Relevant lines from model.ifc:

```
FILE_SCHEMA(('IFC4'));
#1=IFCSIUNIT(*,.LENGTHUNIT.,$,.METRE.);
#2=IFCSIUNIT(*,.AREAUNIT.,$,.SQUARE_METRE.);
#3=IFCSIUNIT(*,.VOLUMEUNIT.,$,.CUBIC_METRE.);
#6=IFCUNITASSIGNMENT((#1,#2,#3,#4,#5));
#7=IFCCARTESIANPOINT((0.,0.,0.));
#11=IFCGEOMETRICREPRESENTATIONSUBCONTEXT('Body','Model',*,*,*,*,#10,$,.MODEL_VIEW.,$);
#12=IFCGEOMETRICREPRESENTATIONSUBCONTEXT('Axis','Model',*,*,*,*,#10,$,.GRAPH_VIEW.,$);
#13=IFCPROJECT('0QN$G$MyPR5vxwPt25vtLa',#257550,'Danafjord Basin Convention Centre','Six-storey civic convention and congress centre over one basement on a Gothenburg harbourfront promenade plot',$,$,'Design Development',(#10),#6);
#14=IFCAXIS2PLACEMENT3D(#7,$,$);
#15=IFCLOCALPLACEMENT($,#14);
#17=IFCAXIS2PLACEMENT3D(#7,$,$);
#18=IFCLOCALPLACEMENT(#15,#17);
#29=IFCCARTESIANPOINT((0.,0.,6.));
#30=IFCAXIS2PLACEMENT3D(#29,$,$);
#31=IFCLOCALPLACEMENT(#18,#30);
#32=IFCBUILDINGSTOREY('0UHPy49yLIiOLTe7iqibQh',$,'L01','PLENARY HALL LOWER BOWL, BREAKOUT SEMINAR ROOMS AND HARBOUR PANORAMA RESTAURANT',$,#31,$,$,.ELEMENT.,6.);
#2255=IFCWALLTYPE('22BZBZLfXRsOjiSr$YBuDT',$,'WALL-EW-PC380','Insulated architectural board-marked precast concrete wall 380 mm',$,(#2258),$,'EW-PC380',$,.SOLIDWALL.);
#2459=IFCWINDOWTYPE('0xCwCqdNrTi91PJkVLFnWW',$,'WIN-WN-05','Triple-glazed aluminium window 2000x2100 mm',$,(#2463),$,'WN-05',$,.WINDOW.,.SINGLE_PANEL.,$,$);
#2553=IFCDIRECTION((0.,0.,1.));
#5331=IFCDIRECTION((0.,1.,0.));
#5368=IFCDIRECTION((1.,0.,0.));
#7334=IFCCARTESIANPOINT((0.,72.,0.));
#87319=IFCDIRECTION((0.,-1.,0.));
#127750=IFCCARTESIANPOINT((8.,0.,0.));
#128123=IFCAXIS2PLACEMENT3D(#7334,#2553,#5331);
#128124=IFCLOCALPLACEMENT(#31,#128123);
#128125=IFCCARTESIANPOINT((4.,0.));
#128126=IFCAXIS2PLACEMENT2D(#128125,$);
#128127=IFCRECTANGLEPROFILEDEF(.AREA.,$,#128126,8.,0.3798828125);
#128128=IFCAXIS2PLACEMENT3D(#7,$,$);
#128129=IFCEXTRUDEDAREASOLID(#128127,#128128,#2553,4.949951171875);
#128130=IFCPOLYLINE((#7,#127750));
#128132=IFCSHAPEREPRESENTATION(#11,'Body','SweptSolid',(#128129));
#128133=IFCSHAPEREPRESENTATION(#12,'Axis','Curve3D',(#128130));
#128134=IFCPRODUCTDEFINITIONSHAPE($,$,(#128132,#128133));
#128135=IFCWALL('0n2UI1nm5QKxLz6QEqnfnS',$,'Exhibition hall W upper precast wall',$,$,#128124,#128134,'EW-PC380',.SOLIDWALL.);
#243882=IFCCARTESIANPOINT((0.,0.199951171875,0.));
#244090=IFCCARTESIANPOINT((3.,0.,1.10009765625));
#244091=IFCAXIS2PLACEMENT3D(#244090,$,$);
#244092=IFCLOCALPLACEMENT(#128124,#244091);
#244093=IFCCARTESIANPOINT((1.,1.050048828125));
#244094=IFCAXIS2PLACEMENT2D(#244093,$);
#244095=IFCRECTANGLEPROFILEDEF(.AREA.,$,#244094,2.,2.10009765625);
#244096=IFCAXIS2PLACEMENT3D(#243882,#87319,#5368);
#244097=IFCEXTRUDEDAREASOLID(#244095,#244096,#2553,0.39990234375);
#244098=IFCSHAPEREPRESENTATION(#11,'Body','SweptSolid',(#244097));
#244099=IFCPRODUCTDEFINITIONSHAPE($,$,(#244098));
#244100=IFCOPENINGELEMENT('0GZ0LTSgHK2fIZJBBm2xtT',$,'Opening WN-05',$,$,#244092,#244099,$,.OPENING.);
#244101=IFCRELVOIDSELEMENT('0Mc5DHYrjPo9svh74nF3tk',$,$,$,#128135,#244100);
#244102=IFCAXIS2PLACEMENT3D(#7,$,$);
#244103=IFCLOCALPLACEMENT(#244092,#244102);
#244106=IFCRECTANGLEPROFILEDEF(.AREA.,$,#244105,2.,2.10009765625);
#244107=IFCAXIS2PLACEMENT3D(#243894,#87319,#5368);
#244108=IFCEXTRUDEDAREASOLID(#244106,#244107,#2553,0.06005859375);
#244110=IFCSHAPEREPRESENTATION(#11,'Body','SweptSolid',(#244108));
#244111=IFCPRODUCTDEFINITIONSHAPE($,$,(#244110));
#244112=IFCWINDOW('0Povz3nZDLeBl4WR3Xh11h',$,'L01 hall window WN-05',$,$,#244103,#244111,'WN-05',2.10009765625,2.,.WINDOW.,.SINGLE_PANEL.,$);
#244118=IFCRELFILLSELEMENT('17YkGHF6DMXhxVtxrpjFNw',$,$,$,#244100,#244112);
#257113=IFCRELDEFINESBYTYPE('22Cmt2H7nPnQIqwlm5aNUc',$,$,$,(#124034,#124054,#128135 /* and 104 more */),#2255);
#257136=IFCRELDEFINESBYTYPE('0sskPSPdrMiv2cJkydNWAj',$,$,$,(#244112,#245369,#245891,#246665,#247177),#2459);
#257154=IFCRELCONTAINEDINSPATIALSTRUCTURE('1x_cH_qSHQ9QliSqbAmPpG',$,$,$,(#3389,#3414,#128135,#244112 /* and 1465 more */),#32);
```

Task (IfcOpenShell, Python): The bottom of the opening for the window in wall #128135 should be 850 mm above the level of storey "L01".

```python
import numpy as np
import ifcopenshell
import ifcopenshell.api.geometry
import ifcopenshell.geom
import ifcopenshell.util.element
import ifcopenshell.util.placement
import ifcopenshell.util.shape
import ifcopenshell.util.unit

model = ifcopenshell.open("model.ifc")
unit_scale = ifcopenshell.util.unit.calculate_unit_scale(model)

window = model.by_guid("0Povz3nZDLeBl4WR3Xh11h")
opening = window.FillsVoids[0].RelatingOpeningElement
storey = ifcopenshell.util.element.get_container(window, ifc_class="IfcBuildingStorey")
level = ifcopenshell.util.placement.get_local_placement(storey.ObjectPlacement)[2, 3]

# The opening's origin need not be at the sill, so measure its lowest point.
shape = ifcopenshell.geom.create_shape(ifcopenshell.geom.settings(), opening)
bottom = ifcopenshell.util.shape.get_shape_bottom_elevation(shape, shape.geometry) / unit_scale
dz = level + 0.85 - bottom

shift = np.array([0.0, 0.0, dz])
# The window is placed relative to its opening, so it follows when the opening moves.
matrix = ifcopenshell.util.placement.get_local_placement(opening.ObjectPlacement)
matrix[:3, 3] += shift
ifcopenshell.api.geometry.edit_object_placement(
    model, product=opening, matrix=matrix, is_si=False, should_transform_children=True
)

print(f"moved by {dz * unit_scale:+.3f} m")

model.write("model-out.ifc")
```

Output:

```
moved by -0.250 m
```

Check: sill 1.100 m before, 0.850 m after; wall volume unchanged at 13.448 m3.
